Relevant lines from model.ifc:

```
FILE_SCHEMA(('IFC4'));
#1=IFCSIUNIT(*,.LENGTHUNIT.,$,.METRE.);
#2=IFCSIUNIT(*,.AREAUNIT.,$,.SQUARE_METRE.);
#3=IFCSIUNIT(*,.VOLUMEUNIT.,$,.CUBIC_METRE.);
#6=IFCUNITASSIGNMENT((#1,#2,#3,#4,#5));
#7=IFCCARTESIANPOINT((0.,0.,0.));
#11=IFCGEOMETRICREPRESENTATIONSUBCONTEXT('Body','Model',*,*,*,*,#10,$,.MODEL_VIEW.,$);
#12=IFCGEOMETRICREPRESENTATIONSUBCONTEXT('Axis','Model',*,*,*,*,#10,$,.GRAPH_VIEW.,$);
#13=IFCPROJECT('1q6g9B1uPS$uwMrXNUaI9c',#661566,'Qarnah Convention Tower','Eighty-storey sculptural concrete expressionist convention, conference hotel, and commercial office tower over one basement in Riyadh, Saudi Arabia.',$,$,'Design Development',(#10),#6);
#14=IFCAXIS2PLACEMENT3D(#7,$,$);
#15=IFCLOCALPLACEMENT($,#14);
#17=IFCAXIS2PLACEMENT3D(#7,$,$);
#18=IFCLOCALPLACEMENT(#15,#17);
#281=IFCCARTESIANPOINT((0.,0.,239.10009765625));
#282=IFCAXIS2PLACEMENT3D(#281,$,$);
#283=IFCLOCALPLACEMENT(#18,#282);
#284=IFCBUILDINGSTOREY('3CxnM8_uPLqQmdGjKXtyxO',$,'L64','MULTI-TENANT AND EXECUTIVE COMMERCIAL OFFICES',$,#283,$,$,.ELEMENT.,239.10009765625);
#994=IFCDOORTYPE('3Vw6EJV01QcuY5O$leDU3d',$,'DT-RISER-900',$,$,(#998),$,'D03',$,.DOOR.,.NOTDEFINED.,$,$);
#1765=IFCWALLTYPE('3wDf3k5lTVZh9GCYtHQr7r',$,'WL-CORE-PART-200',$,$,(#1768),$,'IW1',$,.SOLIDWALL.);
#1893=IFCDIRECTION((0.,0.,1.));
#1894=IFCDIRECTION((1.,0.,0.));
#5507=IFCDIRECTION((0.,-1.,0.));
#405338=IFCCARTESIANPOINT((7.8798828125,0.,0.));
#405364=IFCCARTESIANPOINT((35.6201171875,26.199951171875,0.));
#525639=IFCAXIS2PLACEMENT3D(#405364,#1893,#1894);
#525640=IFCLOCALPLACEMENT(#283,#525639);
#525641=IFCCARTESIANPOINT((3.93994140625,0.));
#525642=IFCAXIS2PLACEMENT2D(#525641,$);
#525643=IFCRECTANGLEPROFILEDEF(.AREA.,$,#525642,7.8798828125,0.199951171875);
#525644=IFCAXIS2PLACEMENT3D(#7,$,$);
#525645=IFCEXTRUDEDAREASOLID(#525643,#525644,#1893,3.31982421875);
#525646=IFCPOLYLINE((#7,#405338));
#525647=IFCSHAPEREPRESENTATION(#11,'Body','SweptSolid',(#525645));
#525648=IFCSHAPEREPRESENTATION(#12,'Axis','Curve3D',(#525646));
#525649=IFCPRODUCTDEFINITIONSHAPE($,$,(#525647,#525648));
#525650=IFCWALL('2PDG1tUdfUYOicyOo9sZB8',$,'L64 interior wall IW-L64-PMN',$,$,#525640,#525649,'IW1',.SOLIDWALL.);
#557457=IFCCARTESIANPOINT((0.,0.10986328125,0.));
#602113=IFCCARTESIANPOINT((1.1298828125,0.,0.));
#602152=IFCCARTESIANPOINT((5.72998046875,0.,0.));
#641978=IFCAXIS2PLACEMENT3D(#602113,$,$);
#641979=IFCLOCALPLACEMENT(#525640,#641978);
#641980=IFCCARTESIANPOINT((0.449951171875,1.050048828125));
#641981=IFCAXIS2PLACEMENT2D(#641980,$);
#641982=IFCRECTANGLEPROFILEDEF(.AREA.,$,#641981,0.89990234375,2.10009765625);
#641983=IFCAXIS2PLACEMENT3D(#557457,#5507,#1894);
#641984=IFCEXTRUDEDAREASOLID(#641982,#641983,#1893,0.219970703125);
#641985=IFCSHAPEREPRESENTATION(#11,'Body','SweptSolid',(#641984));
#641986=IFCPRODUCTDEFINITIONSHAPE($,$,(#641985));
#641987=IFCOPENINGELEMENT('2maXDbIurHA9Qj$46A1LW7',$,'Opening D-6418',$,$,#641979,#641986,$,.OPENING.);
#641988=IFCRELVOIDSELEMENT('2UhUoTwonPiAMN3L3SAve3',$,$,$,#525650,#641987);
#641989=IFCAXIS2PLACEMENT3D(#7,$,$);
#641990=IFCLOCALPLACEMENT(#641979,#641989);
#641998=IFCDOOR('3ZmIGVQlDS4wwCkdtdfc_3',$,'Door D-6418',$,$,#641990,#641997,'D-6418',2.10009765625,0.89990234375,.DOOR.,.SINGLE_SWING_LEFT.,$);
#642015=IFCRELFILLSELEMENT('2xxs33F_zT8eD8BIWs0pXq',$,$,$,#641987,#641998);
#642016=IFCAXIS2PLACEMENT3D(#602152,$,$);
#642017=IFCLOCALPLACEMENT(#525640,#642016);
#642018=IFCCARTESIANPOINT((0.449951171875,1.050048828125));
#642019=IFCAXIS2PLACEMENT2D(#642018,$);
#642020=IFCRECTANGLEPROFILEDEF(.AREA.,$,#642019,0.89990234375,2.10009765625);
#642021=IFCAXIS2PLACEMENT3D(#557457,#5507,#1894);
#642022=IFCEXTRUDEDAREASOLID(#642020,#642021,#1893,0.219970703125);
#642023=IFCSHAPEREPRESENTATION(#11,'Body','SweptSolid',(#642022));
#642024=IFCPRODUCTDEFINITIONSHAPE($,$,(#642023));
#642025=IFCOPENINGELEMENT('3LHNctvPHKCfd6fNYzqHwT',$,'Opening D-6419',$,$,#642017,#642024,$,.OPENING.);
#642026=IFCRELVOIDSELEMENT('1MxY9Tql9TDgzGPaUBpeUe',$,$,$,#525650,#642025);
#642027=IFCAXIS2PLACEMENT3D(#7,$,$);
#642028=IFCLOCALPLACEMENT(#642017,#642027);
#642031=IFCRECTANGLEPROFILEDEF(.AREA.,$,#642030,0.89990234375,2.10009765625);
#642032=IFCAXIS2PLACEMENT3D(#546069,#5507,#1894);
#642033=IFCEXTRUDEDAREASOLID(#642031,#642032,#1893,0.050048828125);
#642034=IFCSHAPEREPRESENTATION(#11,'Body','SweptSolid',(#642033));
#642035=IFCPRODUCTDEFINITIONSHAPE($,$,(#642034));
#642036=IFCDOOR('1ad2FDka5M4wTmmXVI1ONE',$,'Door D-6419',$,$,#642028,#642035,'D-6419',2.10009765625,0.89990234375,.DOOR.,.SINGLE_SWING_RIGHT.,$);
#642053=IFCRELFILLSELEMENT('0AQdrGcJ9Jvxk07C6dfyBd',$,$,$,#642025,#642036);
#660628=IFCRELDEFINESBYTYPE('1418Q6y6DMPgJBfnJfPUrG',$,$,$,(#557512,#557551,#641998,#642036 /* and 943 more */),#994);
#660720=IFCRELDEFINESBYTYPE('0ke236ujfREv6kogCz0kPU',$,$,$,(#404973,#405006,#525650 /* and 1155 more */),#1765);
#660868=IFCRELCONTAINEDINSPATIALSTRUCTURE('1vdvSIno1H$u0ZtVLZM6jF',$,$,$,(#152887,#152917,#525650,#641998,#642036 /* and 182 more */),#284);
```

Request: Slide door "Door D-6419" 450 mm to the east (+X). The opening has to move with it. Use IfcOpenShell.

```python
import ifcopenshell
import ifcopenshell.api.geometry
import ifcopenshell.util.placement
import ifcopenshell.util.unit

model = ifcopenshell.open("model.ifc")
unit_scale = ifcopenshell.util.unit.calculate_unit_scale(model)

door = model.by_id(642036)
opening = door.FillsVoids[0].RelatingOpeningElement
wall = opening.VoidsElements[0].RelatingBuildingElement

wall_matrix = ifcopenshell.util.placement.get_local_placement(wall.ObjectPlacement)
shift = wall_matrix[:3, 0] * 0.45 / unit_scale
before = ifcopenshell.util.placement.get_local_placement(door.ObjectPlacement)[:3, 3].copy()

# The door is placed relative to its opening, so it follows when the opening moves.
matrix = ifcopenshell.util.placement.get_local_placement(opening.ObjectPlacement)
matrix[:3, 3] += shift
ifcopenshell.api.geometry.edit_object_placement(
    model, product=opening, matrix=matrix, is_si=False, should_transform_children=True
)

after = ifcopenshell.util.placement.get_local_placement(door.ObjectPlacement)[:3, 3]
print("door moved by", (after - before).round(3) + 0.0)

model.write("model_edited.ifc")
```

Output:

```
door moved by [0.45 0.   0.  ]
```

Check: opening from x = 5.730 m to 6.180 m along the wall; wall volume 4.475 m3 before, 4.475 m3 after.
